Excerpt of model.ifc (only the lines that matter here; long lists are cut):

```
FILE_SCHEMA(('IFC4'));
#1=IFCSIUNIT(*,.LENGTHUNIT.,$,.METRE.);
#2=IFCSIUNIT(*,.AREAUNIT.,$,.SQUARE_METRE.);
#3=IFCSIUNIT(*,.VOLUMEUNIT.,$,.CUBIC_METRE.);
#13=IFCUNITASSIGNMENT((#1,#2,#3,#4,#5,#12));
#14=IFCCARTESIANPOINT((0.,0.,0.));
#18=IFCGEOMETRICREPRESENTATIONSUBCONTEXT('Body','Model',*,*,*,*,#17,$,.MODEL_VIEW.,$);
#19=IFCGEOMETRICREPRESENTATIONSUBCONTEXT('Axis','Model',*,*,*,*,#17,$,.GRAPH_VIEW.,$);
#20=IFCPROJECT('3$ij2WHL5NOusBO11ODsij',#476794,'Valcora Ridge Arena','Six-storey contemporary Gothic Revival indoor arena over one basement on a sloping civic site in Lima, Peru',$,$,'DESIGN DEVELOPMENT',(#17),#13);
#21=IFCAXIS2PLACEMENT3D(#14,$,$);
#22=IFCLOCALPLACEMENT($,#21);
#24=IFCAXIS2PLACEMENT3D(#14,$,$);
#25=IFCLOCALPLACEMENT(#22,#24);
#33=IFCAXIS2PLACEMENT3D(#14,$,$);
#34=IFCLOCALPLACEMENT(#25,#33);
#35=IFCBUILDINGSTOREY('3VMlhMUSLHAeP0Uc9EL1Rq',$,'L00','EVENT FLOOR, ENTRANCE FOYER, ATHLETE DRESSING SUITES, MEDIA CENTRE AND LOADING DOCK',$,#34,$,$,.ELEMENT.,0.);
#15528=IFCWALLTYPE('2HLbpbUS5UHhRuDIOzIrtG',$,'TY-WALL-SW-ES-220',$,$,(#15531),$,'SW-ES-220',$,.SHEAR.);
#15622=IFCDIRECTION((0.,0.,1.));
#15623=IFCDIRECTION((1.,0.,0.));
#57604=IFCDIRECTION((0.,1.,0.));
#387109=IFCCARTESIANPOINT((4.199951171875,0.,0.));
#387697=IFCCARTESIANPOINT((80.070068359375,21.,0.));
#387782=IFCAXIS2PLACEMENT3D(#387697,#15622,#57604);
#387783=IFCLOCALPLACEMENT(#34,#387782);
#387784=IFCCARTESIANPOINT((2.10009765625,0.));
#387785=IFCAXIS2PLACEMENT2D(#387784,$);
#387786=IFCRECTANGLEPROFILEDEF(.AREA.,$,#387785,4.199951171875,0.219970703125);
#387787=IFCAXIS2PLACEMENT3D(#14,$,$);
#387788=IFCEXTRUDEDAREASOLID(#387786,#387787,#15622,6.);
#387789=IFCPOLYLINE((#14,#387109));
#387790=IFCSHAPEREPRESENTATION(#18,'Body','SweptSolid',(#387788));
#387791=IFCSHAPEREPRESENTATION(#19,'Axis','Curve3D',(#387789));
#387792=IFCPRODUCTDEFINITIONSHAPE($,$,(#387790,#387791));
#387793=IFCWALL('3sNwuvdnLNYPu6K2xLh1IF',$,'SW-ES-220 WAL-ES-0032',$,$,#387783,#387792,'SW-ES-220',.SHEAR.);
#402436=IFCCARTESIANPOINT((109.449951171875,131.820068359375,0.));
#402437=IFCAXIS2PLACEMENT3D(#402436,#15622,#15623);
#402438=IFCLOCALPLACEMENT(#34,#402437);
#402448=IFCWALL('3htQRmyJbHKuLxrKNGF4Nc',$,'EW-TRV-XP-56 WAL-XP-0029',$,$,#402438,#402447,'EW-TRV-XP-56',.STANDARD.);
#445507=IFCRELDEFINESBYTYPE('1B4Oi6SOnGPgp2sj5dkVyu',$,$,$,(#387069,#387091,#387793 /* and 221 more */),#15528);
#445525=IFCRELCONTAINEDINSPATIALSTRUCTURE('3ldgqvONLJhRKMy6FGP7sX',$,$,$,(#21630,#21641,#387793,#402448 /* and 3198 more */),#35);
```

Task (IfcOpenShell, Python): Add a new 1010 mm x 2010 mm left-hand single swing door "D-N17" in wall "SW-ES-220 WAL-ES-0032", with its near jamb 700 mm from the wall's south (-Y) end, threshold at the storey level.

```python
import numpy as np
import ifcopenshell
import ifcopenshell.api.feature
import ifcopenshell.api.geometry
import ifcopenshell.api.root
import ifcopenshell.api.spatial
import ifcopenshell.geom
import ifcopenshell.util.element
import ifcopenshell.util.placement
import ifcopenshell.util.representation
import ifcopenshell.util.shape
import ifcopenshell.util.unit

model = ifcopenshell.open("model.ifc")
unit_scale = ifcopenshell.util.unit.calculate_unit_scale(model)
settings = ifcopenshell.geom.settings()


def volume(element):
    """Net volume in cubic metres, openings subtracted."""
    shape = ifcopenshell.geom.create_shape(settings, element)
    return ifcopenshell.util.shape.get_volume(shape.geometry)


wall = model.by_guid("3sNwuvdnLNYPu6K2xLh1IF")
storey = ifcopenshell.util.element.get_container(wall, ifc_class="IfcBuildingStorey")
context = ifcopenshell.util.representation.get_context(model, "Model", "Body", "MODEL_VIEW")
before = volume(wall)

width, height, from_end, sill = 1.01, 2.01, 0.7, 0.0  # metres

# The wall runs along its own X axis, and the end named is its -X end.
wall_shape = ifcopenshell.geom.create_shape(settings, wall)
x, y, z = ifcopenshell.util.shape.get_vertices(wall_shape.geometry).T
start = x.min() + from_end
face, thickness = float(y.min()), float(y.max() - y.min())
wall_matrix = ifcopenshell.util.placement.get_local_placement(wall.ObjectPlacement)
level = ifcopenshell.util.placement.get_local_placement(storey.ObjectPlacement)[2, 3]


def in_wall(x, y):
    """Placement at x, y metres in the wall's axes, at sill height."""
    matrix = wall_matrix.copy()
    matrix[:, 3] = wall_matrix @ np.array([x / unit_scale, y / unit_scale, 0.0, 1.0])
    matrix[2, 3] = level + sill / unit_scale
    return matrix


# Opening: a box that overshoots both wall faces by 50 mm.
opening = ifcopenshell.api.root.create_entity(model, ifc_class="IfcOpeningElement", predefined_type="OPENING")
box = ifcopenshell.api.geometry.add_wall_representation(
    model, context=context, length=width, height=height, thickness=thickness + 0.1
)
ifcopenshell.api.geometry.assign_representation(model, product=opening, representation=box)
ifcopenshell.api.geometry.edit_object_placement(model, product=opening, matrix=in_wall(start, face - 0.05), is_si=False)
ifcopenshell.api.feature.add_feature(model, feature=opening, element=wall)

door = ifcopenshell.api.root.create_entity(model, ifc_class="IfcDoor", name="D-N17", predefined_type="DOOR")
door.OverallWidth, door.OverallHeight = width / unit_scale, height / unit_scale
door.OperationType = "SINGLE_SWING_LEFT"
body = ifcopenshell.api.geometry.add_door_representation(
    model,
    context=context,
    overall_width=door.OverallWidth,
    overall_height=door.OverallHeight,
    operation_type="SINGLE_SWING_LEFT",
    lining_properties={"LiningDepth": thickness / unit_scale, "ThresholdDepth": thickness / unit_scale},
)
ifcopenshell.api.geometry.assign_representation(model, product=door, representation=body)
ifcopenshell.api.spatial.assign_container(model, products=[door], relating_structure=storey)
ifcopenshell.api.feature.add_filling(model, opening=opening, element=door)

# The lining spans the wall, so the door starts at the wall face.
ifcopenshell.api.geometry.edit_object_placement(model, product=door, matrix=in_wall(start, face), is_si=False)

after = volume(wall)

print(f"wall volume {before:.3f} -> {after:.3f} m3")

model.write("model-out.ifc")
```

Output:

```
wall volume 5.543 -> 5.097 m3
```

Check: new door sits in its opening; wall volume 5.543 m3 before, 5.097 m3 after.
